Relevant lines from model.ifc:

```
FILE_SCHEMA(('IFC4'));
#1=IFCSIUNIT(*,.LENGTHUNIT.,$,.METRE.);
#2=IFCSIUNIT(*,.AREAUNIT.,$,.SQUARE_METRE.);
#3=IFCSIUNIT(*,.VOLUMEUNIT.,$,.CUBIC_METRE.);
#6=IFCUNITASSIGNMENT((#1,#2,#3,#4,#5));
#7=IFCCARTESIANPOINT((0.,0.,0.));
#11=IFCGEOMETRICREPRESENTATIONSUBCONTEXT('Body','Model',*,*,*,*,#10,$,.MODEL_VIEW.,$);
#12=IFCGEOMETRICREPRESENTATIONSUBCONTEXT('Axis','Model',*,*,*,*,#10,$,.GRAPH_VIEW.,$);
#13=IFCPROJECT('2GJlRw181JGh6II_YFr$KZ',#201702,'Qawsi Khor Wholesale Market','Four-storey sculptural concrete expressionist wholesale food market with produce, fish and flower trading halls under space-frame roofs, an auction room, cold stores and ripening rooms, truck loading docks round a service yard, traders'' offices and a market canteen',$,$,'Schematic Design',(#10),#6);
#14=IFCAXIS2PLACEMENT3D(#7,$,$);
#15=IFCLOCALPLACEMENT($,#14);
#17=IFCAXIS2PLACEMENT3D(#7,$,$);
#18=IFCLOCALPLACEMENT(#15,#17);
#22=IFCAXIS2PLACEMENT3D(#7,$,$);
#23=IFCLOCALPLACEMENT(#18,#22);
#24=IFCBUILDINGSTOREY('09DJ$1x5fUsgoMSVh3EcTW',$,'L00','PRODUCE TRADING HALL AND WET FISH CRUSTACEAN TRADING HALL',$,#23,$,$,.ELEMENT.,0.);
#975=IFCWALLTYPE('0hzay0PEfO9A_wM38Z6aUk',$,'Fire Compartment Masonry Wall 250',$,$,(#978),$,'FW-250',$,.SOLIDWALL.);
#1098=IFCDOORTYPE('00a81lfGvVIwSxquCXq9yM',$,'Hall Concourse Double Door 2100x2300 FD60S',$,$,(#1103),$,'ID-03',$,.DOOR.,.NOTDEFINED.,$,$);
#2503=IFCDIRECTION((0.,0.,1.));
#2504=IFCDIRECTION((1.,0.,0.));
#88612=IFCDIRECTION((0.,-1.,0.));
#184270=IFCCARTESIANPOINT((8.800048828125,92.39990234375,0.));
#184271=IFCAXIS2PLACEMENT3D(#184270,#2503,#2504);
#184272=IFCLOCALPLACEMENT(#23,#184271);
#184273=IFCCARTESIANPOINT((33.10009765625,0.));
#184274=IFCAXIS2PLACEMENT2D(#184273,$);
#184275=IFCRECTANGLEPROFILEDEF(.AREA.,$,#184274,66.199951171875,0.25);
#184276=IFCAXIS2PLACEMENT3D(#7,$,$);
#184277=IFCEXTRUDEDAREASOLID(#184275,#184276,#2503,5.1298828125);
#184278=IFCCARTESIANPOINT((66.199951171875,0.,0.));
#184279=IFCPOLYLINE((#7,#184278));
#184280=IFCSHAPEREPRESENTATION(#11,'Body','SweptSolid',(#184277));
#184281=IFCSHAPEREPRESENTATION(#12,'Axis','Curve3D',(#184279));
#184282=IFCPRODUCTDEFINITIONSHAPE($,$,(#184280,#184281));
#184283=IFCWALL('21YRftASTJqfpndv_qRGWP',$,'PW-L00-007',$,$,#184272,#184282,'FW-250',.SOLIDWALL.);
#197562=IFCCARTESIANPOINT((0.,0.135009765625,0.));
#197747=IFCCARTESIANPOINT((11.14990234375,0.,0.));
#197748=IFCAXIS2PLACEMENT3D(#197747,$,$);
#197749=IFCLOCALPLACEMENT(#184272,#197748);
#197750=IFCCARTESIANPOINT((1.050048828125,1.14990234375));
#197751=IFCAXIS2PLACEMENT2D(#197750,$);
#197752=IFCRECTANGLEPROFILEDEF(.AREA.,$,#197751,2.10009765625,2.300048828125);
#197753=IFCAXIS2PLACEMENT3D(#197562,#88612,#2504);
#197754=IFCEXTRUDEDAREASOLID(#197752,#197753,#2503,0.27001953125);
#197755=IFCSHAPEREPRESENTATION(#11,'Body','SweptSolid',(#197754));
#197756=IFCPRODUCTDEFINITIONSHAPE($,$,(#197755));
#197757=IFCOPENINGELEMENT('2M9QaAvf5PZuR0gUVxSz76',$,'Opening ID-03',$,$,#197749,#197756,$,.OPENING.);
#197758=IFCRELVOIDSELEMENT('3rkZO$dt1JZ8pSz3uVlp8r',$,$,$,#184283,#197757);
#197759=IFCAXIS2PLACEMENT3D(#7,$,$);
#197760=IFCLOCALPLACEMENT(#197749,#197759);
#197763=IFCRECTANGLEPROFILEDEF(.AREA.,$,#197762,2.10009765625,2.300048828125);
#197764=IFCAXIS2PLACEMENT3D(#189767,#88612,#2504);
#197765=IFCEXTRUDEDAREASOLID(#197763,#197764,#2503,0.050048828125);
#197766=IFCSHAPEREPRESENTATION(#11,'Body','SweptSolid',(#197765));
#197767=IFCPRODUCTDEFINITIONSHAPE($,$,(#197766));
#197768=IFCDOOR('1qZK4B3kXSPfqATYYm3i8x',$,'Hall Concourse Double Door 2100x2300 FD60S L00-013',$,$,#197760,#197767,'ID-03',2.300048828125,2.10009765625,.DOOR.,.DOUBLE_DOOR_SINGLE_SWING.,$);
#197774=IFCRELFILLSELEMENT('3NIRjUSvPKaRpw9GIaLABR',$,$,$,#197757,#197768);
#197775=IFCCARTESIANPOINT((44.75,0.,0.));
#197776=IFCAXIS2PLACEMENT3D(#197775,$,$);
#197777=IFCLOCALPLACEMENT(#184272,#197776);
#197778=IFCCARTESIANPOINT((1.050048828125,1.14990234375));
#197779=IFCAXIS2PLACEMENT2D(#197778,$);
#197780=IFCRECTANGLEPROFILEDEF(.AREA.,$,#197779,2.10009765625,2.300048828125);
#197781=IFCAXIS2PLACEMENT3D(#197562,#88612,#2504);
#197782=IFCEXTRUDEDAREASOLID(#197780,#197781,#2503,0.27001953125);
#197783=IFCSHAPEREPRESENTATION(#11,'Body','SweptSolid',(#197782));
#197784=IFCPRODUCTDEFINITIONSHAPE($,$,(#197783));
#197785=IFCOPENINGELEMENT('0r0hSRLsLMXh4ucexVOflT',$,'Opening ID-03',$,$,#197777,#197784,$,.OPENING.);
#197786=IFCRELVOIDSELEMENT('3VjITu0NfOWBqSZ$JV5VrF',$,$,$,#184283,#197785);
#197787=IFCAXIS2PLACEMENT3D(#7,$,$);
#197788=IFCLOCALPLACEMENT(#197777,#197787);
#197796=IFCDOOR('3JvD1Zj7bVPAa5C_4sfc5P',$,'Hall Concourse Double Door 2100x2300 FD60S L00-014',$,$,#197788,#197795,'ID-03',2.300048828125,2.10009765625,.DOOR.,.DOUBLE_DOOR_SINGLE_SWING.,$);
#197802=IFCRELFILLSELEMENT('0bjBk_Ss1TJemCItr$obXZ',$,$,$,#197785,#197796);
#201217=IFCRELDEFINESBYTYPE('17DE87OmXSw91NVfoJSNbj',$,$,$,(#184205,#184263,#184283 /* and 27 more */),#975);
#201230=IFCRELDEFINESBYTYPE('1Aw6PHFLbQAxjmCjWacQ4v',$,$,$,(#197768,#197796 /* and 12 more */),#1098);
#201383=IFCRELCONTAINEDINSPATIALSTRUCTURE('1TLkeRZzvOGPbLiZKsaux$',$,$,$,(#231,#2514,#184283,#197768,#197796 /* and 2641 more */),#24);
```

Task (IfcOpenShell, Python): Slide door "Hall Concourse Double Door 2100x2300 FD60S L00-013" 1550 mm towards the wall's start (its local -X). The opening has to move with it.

```python
import ifcopenshell
import ifcopenshell.api.geometry
import ifcopenshell.util.placement

model = ifcopenshell.open("model.ifc")

door = model.by_guid("1qZK4B3kXSPfqATYYm3i8x")
opening = door.FillsVoids[0].RelatingOpeningElement
wall = opening.VoidsElements[0].RelatingBuildingElement

wall_matrix = ifcopenshell.util.placement.get_local_placement(wall.ObjectPlacement)
shift = wall_matrix[:3, 0] * -1.55
before = ifcopenshell.util.placement.get_local_placement(door.ObjectPlacement)[:3, 3].copy()

# The door is placed relative to its opening, so it follows when the opening moves.
matrix = ifcopenshell.util.placement.get_local_placement(opening.ObjectPlacement)
matrix[:3, 3] += shift
ifcopenshell.api.geometry.edit_object_placement(
    model, product=opening, matrix=matrix, is_si=False, should_transform_children=True
)

after = ifcopenshell.util.placement.get_local_placement(door.ObjectPlacement)[:3, 3]
print("door moved by", (after - before).round(3) + 0.0)

model.write("model-out.ifc")
```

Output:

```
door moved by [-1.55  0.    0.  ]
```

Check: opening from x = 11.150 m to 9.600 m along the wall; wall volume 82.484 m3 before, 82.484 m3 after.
